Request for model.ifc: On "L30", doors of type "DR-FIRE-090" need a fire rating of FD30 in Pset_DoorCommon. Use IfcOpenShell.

First a look at what the model holds.

```python
import ifcopenshell
import ifcopenshell.util.element

model = ifcopenshell.open("model.ifc")
print(model.schema)
storey = next(s for s in model.by_type("IfcBuildingStorey") if s.Name == "L30")
doors = [e for e in ifcopenshell.util.element.get_decomposition(storey) if e.is_a("IfcDoor")]
seen = {}
for e in doors:
    element_type = ifcopenshell.util.element.get_type(e)
    key = (element_type.Name if element_type != e and element_type else None, ifcopenshell.util.element.get_pset(e, "Pset_DoorCommon", "FireRating"))
    seen[key] = seen.get(key, 0) + 1
for (name, value), count in sorted(seen.items(), key=str):
    print(count, "x", name, "|", value)
```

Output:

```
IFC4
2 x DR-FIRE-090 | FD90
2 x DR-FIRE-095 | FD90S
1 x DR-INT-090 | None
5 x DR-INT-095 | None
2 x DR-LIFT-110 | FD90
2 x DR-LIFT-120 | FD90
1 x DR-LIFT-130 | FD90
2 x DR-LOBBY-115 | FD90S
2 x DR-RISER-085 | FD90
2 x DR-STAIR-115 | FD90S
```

```python
import ifcopenshell
import ifcopenshell.api.pset
import ifcopenshell.util.element

model = ifcopenshell.open("model.ifc")

storey = next(s for s in model.by_type("IfcBuildingStorey") if s.Name == "L30")
doors = [e for e in ifcopenshell.util.element.get_decomposition(storey) if e.is_a("IfcDoor")]

count = 0
for e in doors:
    element_type = ifcopenshell.util.element.get_type(e)
    if element_type in (None, e) or element_type.Name != "DR-FIRE-090":
        continue
    found = ifcopenshell.util.element.get_pset(e, "Pset_DoorCommon", should_inherit=False)
    if found:
        pset = model.by_id(found["id"])
        if len(ifcopenshell.util.element.get_elements_by_pset(pset)) > 1:
            pset = ifcopenshell.api.pset.unshare_pset(model, products=[e], pset=pset)[0]
    else:
        pset = ifcopenshell.api.pset.add_pset(model, product=e, name="Pset_DoorCommon")
    ifcopenshell.api.pset.edit_pset(model, pset=pset, properties={"FireRating": "FD30"})
    count += 1

print(count, "doors updated")

model.write("model_v2.ifc")
```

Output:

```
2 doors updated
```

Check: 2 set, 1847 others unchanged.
